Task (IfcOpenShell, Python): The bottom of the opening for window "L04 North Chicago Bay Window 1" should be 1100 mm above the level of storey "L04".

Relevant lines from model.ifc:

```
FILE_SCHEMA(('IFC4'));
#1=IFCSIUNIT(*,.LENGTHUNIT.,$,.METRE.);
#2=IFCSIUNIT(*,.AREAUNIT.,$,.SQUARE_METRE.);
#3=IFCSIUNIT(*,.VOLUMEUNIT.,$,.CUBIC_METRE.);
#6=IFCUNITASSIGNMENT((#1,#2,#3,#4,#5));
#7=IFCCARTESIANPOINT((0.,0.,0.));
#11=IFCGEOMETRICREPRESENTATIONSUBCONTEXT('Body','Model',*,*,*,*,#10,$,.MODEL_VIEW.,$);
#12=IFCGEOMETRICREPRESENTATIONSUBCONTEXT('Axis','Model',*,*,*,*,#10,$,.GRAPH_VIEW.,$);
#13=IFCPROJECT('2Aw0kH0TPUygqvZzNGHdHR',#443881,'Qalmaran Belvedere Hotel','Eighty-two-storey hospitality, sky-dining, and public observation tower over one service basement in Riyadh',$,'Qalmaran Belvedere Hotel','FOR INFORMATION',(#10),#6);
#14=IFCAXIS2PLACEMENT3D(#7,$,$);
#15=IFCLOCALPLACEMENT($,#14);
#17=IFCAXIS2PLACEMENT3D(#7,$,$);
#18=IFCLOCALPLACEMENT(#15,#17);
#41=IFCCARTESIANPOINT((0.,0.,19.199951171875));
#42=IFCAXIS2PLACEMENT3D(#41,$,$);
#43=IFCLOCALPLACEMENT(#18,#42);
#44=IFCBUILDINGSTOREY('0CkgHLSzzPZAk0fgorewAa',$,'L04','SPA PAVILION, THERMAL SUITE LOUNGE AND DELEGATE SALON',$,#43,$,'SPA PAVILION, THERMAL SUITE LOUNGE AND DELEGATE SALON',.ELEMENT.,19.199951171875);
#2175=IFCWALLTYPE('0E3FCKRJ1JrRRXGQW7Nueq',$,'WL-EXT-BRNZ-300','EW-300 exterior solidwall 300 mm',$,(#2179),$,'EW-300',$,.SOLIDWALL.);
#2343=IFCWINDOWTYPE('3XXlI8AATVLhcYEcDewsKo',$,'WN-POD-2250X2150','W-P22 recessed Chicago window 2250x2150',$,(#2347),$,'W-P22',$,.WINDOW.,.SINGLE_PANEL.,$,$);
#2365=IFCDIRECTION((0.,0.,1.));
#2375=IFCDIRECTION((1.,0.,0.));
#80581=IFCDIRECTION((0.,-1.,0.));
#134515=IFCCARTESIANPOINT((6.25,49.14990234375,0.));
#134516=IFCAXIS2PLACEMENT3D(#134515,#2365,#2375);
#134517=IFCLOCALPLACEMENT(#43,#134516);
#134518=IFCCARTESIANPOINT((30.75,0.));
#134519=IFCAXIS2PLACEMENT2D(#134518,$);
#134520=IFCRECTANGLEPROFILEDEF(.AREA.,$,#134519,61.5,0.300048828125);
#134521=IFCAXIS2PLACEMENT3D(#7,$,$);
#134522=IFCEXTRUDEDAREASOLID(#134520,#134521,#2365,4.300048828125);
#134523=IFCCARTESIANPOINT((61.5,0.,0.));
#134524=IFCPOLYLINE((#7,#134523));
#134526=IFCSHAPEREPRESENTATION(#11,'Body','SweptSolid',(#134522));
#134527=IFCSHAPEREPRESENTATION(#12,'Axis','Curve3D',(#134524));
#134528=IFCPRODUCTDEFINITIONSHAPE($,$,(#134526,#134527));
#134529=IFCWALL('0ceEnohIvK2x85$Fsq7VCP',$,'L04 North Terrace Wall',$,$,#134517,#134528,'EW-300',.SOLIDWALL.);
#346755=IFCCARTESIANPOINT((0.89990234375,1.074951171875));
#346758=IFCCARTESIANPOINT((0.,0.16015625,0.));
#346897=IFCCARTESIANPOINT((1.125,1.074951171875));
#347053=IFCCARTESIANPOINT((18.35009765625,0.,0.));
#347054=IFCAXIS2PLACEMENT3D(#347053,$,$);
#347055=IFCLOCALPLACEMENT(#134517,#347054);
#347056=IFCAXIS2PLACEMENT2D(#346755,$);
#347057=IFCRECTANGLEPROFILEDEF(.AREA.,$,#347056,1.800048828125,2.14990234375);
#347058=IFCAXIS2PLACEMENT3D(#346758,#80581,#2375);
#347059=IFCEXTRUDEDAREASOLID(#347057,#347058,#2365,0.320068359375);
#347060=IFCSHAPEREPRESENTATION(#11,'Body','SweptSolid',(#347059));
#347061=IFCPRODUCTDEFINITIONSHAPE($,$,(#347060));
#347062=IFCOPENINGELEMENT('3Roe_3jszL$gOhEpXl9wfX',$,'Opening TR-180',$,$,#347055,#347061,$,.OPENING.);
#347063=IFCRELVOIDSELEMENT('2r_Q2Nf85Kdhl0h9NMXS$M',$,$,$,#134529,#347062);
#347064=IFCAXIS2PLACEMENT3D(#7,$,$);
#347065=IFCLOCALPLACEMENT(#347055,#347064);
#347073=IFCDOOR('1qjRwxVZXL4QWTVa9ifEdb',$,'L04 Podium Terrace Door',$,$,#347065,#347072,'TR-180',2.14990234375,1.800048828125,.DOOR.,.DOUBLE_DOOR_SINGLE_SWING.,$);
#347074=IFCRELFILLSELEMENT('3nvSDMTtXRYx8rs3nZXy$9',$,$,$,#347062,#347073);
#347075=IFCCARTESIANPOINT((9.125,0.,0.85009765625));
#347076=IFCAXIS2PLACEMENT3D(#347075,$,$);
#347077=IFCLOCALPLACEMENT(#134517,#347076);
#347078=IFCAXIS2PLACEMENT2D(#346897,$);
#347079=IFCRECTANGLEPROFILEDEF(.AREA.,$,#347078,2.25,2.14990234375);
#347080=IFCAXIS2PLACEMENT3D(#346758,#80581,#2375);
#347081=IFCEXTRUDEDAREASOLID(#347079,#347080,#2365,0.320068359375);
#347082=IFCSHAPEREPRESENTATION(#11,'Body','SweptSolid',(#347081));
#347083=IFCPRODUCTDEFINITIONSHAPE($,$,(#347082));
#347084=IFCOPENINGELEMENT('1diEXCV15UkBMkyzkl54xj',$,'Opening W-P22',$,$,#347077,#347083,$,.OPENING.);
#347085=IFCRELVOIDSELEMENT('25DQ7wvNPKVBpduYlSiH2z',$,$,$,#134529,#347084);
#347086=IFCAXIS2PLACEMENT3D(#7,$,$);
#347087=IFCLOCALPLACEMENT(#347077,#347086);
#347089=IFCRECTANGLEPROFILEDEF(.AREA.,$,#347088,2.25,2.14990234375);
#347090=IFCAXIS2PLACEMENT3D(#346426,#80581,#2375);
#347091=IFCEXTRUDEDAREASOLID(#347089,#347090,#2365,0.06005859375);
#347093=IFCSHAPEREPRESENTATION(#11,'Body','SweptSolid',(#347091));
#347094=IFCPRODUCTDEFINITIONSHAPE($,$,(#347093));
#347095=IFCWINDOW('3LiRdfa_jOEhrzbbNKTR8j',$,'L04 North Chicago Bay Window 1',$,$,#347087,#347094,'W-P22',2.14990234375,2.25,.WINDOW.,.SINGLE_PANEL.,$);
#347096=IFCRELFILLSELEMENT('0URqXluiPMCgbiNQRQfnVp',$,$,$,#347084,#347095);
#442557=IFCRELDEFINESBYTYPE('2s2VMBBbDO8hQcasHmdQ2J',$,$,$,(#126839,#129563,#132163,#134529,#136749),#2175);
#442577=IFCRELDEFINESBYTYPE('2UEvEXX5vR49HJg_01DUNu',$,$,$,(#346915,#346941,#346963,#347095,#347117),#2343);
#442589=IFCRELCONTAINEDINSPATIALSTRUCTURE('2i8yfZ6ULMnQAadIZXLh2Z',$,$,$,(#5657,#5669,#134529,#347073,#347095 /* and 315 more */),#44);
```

```python
import numpy as np
import ifcopenshell
import ifcopenshell.api.geometry
import ifcopenshell.geom
import ifcopenshell.util.element
import ifcopenshell.util.placement
import ifcopenshell.util.shape
import ifcopenshell.util.unit

model = ifcopenshell.open("model.ifc")
unit_scale = ifcopenshell.util.unit.calculate_unit_scale(model)

window = model.by_guid("3LiRdfa_jOEhrzbbNKTR8j")
opening = window.FillsVoids[0].RelatingOpeningElement
storey = ifcopenshell.util.element.get_container(window, ifc_class="IfcBuildingStorey")
level = ifcopenshell.util.placement.get_local_placement(storey.ObjectPlacement)[2, 3]

# The opening's origin need not be at the sill, so measure its lowest point.
shape = ifcopenshell.geom.create_shape(ifcopenshell.geom.settings(), opening)
bottom = ifcopenshell.util.shape.get_shape_bottom_elevation(shape, shape.geometry) / unit_scale
dz = level + 1.1 / unit_scale - bottom

shift = np.array([0.0, 0.0, dz])
# The window is placed relative to its opening, so it follows when the opening moves.
matrix = ifcopenshell.util.placement.get_local_placement(opening.ObjectPlacement)
matrix[:3, 3] += shift
ifcopenshell.api.geometry.edit_object_placement(
    model, product=opening, matrix=matrix, is_si=False, should_transform_children=True
)

print(f"moved by {dz * unit_scale:+.3f} m")

model.write("model_rev.ifc")
```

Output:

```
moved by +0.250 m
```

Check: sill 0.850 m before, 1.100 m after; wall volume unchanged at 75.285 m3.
